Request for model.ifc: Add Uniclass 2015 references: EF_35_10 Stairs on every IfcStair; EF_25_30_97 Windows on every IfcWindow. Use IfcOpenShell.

First a look at what the model holds.

```python
import ifcopenshell

model = ifcopenshell.open("model.ifc")
print(model.schema)
print("classifications:", [c.Name for c in model.by_type("IfcClassification")])
for ifc_class in ("IfcDoor", "IfcRoof", "IfcStair", "IfcWall", "IfcWindow"):
    print(ifc_class, len(model.by_type(ifc_class)))
```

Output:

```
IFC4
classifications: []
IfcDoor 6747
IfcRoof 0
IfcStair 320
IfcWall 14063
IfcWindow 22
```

```python
import ifcopenshell
import ifcopenshell.api.classification

model = ifcopenshell.open("model.ifc")

system = ifcopenshell.api.classification.add_classification(model, classification="Uniclass 2015")

codes = {
    "IfcStair": ("EF_35_10", "Stairs"),
    "IfcWindow": ("EF_25_30_97", "Windows"),
}
for ifc_class, (code, name) in codes.items():
    products = model.by_type(ifc_class)
    ifcopenshell.api.classification.add_reference(
        model, products=products, classification=system, identification=code, name=name
    )
    print(code, len(products))

model.write("model_edited.ifc")
```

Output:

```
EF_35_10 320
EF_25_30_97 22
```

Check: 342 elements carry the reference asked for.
